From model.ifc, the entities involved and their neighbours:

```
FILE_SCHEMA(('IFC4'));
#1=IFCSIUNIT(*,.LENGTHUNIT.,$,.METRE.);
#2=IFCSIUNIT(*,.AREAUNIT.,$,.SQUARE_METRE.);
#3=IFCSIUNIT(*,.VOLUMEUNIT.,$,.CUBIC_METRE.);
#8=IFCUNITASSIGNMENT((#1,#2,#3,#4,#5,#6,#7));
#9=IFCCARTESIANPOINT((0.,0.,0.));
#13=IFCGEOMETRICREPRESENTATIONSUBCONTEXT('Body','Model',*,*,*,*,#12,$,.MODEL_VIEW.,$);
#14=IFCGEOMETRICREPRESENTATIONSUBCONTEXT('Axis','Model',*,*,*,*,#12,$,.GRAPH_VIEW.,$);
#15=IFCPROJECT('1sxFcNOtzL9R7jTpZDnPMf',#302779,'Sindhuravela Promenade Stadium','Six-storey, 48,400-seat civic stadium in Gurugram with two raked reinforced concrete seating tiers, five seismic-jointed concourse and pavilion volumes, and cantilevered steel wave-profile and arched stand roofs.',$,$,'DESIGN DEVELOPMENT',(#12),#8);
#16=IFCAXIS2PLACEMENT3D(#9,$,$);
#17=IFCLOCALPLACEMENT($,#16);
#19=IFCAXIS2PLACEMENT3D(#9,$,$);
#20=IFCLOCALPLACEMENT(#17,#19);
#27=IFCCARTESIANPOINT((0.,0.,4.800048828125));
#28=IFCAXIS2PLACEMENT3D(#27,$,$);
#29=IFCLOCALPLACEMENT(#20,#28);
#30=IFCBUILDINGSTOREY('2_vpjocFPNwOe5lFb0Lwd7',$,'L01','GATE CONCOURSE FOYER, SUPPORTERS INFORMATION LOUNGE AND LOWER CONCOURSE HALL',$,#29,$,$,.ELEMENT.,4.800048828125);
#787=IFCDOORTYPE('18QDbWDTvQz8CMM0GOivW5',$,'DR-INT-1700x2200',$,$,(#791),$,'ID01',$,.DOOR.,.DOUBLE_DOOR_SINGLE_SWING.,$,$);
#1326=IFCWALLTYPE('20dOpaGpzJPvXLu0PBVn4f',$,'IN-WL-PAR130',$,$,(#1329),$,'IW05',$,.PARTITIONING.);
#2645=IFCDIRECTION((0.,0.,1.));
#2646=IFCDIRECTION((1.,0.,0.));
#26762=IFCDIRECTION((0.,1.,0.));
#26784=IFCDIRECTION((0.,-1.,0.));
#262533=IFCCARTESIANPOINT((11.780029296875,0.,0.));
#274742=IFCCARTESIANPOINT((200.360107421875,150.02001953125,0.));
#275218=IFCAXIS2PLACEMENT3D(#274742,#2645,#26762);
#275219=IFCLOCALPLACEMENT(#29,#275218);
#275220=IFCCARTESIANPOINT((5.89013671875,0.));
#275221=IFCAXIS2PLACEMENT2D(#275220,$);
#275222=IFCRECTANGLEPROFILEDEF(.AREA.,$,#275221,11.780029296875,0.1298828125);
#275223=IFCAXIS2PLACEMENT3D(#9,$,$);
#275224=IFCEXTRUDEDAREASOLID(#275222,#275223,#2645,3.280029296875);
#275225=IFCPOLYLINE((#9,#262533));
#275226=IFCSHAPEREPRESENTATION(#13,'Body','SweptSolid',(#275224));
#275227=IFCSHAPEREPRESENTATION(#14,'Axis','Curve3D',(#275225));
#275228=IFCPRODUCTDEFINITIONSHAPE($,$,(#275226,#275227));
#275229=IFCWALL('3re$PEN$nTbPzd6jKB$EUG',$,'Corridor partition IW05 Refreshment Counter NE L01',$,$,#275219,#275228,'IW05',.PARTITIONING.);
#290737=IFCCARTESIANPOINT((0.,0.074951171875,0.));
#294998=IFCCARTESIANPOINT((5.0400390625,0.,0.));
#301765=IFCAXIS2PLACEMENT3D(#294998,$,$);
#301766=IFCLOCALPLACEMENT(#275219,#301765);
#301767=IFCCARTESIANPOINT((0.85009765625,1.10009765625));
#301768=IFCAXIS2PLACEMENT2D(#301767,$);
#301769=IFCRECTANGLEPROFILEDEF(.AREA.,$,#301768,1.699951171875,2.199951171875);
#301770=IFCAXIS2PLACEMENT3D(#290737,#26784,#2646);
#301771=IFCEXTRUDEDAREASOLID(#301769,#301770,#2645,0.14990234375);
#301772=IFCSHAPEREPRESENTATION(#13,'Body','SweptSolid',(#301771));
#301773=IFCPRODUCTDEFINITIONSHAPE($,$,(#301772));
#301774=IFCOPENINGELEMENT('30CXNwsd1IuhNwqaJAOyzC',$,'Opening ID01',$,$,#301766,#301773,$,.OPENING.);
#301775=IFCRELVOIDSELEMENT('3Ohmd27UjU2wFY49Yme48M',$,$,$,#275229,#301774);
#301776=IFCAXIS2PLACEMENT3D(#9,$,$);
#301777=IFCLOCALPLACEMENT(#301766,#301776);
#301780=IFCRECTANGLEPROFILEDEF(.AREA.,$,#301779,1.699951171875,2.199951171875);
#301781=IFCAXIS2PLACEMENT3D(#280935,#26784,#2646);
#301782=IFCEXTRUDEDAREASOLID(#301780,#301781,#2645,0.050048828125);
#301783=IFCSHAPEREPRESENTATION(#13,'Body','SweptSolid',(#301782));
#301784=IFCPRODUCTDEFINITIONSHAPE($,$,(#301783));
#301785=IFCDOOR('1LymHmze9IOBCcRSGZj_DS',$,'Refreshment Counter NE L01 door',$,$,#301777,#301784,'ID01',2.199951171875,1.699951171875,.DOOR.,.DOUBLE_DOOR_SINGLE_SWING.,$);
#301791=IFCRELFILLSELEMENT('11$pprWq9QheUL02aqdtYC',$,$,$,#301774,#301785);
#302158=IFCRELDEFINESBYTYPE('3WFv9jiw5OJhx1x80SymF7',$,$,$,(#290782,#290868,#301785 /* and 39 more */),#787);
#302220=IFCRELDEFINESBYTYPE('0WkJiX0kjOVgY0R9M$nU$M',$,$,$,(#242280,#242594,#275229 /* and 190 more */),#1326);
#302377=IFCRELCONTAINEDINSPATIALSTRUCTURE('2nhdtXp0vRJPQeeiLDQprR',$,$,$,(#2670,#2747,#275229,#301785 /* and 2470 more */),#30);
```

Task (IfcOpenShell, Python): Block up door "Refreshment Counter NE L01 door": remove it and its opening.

```python
import ifcopenshell
import ifcopenshell.api.feature
import ifcopenshell.api.root
import ifcopenshell.geom
import ifcopenshell.util.shape

model = ifcopenshell.open("model.ifc")
settings = ifcopenshell.geom.settings()


def volume(element):
    """Net volume in cubic metres, openings subtracted."""
    shape = ifcopenshell.geom.create_shape(settings, element)
    return ifcopenshell.util.shape.get_volume(shape.geometry)


door = model.by_guid("1LymHmze9IOBCcRSGZj_DS")
opening = door.FillsVoids[0].RelatingOpeningElement
wall = opening.VoidsElements[0].RelatingBuildingElement
before = volume(wall)

ifcopenshell.api.root.remove_product(model, product=door)
ifcopenshell.api.feature.remove_feature(model, feature=opening)

after = volume(wall)

print(f"wall volume {before:.3f} -> {after:.3f} m3")

model.write("model-out.ifc")
```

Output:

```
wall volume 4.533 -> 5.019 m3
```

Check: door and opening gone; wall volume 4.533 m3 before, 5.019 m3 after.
